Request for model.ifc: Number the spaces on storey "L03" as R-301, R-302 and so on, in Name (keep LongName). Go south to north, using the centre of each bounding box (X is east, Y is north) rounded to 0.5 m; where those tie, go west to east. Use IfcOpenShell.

First a look at what the model holds.

```python
import ifcopenshell
import ifcopenshell.util.element
import ifcopenshell.util.placement

model = ifcopenshell.open("model.ifc")
print(model.schema)
storey = next(s for s in model.by_type("IfcBuildingStorey") if s.Name == "L03")
spaces = [e for e in ifcopenshell.util.element.get_decomposition(storey) if e.is_a("IfcSpace")]
for e in sorted(spaces, key=lambda e: e.id()):
    origin = ifcopenshell.util.placement.get_local_placement(e.ObjectPlacement)[:3, 3]
    print(e.id(), e.Name, e.LongName, origin.round(2) + 0.0, sep=" | ")
```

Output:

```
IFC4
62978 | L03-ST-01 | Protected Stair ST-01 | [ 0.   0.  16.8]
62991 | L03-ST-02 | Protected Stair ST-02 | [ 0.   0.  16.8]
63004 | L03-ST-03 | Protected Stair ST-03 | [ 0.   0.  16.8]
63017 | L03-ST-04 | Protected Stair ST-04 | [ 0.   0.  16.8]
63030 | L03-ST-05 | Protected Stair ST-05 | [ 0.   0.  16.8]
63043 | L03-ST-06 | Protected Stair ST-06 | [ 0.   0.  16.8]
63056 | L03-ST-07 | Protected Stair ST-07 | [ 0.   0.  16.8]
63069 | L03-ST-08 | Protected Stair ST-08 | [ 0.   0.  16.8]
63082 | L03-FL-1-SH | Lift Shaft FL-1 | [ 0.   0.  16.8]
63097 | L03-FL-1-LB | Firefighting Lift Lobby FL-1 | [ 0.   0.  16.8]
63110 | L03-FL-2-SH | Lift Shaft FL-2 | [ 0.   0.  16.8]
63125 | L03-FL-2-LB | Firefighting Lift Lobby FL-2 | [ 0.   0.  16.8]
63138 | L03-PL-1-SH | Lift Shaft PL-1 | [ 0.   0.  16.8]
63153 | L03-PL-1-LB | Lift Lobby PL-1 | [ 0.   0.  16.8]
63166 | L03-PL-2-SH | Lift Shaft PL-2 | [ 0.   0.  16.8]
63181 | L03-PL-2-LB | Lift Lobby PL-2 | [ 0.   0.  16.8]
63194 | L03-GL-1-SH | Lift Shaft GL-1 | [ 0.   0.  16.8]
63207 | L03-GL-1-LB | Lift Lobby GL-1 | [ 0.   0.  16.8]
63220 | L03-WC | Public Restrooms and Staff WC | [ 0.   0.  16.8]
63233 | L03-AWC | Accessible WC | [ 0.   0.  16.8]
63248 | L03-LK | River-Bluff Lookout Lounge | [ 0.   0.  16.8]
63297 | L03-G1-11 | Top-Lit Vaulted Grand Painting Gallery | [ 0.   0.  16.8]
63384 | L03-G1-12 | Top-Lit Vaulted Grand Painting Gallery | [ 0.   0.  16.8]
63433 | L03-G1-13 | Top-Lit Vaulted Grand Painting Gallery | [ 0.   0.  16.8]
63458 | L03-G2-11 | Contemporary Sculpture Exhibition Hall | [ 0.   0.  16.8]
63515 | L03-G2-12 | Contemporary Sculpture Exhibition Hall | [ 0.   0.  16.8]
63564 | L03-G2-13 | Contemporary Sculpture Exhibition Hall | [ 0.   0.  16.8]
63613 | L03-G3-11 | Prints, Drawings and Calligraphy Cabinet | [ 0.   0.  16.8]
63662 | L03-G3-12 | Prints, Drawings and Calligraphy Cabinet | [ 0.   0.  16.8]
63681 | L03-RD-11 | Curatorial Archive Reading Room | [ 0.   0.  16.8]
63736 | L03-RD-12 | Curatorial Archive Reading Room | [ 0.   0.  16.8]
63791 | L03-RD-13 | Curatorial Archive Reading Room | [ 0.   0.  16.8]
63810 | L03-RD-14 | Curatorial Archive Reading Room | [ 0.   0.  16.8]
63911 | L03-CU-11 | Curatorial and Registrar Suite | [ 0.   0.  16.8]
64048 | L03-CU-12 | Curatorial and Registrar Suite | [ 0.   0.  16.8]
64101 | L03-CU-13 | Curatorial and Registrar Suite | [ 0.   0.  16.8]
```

```python
import ifcopenshell
import ifcopenshell.geom
import ifcopenshell.util.element
import ifcopenshell.util.shape

model = ifcopenshell.open("model.ifc")
settings = ifcopenshell.geom.settings()
settings.set("use-world-coords", True)


def centre(element):
    shape = ifcopenshell.geom.create_shape(settings, element)
    return ifcopenshell.util.shape.get_bbox_centroid(shape.geometry)


storey = next(s for s in model.by_type("IfcBuildingStorey") if s.Name == "L03")
spaces = [e for e in ifcopenshell.util.element.get_decomposition(storey) if e.is_a("IfcSpace")]

# Insertion points can sit at a corner or the storey origin, so sort by the geometry (in metres).
centres = {e: centre(e) for e in spaces}
spaces.sort(key=lambda e: (round(centres[e][1] / 0.5), centres[e][0]))

for i, e in enumerate(spaces, start=1):
    number = f"R-3{i:02d}"
    e.Name = number
    print(e.id(), number)

model.write("model_v2.ifc")
```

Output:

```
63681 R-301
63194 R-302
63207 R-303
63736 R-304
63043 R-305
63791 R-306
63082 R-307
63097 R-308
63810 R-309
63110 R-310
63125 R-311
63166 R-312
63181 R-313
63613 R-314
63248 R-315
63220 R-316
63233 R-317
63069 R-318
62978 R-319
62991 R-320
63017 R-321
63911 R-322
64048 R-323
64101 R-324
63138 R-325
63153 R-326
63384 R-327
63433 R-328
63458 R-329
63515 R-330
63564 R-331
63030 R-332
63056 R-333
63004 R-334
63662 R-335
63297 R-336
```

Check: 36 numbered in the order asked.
